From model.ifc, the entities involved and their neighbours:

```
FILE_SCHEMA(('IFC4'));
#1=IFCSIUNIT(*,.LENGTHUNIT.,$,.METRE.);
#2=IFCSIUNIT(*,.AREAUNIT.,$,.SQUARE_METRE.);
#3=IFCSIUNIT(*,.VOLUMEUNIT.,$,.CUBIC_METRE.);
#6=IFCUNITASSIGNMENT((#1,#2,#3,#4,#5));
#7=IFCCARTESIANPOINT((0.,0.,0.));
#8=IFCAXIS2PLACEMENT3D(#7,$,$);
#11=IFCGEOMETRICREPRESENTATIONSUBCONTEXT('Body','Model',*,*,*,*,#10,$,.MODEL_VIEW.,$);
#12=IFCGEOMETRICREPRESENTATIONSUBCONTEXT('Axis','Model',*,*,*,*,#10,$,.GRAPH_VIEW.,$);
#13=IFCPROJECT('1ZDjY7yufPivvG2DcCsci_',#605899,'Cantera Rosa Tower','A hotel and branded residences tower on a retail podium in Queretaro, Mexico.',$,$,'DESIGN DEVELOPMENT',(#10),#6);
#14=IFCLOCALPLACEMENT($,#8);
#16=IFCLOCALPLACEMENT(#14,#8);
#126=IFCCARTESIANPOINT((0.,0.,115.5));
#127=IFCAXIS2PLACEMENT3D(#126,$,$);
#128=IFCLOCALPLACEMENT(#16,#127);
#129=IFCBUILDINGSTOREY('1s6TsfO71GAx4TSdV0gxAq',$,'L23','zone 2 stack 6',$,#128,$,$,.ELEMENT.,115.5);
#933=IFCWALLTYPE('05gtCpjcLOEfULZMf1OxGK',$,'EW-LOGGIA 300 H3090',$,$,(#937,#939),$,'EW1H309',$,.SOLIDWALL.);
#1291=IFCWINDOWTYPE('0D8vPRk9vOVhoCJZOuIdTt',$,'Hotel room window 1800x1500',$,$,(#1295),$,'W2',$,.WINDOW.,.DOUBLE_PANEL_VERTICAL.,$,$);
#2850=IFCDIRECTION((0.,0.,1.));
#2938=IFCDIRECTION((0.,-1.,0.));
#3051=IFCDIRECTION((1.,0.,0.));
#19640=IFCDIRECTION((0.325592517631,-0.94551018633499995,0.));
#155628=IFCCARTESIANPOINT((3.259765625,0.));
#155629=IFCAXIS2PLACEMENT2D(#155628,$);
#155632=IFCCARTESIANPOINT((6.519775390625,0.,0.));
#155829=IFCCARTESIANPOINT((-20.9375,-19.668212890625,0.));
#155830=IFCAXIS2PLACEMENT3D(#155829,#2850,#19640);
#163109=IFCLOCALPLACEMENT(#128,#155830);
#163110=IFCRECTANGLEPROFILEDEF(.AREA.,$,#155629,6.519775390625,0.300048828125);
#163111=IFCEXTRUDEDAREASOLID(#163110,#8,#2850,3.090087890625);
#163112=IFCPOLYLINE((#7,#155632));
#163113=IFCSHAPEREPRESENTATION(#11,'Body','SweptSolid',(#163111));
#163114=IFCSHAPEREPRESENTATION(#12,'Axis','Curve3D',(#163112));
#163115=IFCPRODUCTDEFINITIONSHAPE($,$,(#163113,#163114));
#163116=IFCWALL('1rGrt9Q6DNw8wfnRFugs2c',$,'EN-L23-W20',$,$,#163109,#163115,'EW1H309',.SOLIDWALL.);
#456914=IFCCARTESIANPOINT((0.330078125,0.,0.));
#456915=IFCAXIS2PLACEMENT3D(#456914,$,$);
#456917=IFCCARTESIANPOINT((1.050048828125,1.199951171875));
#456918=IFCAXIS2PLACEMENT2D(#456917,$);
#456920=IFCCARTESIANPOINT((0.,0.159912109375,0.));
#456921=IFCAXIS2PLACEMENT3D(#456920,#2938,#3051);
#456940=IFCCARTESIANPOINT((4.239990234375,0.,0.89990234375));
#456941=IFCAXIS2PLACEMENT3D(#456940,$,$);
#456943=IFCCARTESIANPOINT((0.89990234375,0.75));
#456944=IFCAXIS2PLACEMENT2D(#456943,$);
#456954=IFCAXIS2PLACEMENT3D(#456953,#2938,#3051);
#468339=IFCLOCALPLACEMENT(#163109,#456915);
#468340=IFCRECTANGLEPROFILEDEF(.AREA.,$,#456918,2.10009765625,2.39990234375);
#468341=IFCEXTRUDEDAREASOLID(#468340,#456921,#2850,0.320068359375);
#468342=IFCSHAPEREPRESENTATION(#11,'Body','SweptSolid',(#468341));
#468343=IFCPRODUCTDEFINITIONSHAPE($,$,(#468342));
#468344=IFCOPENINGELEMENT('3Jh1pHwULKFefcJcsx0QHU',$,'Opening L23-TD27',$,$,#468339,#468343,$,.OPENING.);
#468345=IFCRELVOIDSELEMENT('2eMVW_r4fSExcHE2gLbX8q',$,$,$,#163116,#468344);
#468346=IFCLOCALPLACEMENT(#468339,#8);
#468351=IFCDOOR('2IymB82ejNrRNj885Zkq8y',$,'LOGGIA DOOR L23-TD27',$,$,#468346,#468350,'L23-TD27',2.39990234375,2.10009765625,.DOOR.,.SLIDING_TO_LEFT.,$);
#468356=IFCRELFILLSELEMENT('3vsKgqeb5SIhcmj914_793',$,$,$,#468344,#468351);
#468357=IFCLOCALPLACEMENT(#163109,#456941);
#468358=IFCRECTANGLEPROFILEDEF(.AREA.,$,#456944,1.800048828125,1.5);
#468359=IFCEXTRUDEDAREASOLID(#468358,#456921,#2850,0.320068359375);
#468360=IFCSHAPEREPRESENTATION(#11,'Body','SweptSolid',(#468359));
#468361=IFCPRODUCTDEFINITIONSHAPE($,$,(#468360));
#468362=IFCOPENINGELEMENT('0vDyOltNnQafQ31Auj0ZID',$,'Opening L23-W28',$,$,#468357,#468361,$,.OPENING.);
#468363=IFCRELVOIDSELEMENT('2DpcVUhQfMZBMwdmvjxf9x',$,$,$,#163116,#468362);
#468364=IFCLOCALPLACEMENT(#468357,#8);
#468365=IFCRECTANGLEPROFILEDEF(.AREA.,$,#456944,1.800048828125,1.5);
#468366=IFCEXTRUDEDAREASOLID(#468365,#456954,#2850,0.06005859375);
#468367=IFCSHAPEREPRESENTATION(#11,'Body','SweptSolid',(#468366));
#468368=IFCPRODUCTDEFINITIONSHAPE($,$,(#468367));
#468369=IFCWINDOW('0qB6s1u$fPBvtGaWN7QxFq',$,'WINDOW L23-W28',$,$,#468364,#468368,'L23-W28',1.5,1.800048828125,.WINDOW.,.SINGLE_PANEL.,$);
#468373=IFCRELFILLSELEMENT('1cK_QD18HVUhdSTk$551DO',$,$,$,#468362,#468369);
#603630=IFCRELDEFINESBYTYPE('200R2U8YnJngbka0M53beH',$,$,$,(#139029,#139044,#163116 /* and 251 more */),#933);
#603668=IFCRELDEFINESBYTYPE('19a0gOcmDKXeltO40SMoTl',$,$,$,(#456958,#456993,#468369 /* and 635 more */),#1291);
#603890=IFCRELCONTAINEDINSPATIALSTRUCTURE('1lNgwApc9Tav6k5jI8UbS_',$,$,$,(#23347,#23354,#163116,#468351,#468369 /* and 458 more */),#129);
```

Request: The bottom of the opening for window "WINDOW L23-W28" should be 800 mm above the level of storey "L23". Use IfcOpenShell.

```python
import numpy as np
import ifcopenshell
import ifcopenshell.api.geometry
import ifcopenshell.geom
import ifcopenshell.util.element
import ifcopenshell.util.placement
import ifcopenshell.util.shape
import ifcopenshell.util.unit

model = ifcopenshell.open("model.ifc")
unit_scale = ifcopenshell.util.unit.calculate_unit_scale(model)

window = model.by_id(468369)
opening = window.FillsVoids[0].RelatingOpeningElement
storey = ifcopenshell.util.element.get_container(window, ifc_class="IfcBuildingStorey")
level = ifcopenshell.util.placement.get_local_placement(storey.ObjectPlacement)[2, 3]

# The opening's origin need not be at the sill, so measure its lowest point.
shape = ifcopenshell.geom.create_shape(ifcopenshell.geom.settings(), opening)
bottom = ifcopenshell.util.shape.get_shape_bottom_elevation(shape, shape.geometry) / unit_scale
dz = level + 0.8 - bottom

shift = np.array([0.0, 0.0, dz])
# The window is placed relative to its opening, so it follows when the opening moves.
matrix = ifcopenshell.util.placement.get_local_placement(opening.ObjectPlacement)
matrix[:3, 3] += shift
ifcopenshell.api.geometry.edit_object_placement(
    model, product=opening, matrix=matrix, is_si=False, should_transform_children=True
)

print(f"moved by {dz * unit_scale:+.3f} m")

model.write("model_rev.ifc")
```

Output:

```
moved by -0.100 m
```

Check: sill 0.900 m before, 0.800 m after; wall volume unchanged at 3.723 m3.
